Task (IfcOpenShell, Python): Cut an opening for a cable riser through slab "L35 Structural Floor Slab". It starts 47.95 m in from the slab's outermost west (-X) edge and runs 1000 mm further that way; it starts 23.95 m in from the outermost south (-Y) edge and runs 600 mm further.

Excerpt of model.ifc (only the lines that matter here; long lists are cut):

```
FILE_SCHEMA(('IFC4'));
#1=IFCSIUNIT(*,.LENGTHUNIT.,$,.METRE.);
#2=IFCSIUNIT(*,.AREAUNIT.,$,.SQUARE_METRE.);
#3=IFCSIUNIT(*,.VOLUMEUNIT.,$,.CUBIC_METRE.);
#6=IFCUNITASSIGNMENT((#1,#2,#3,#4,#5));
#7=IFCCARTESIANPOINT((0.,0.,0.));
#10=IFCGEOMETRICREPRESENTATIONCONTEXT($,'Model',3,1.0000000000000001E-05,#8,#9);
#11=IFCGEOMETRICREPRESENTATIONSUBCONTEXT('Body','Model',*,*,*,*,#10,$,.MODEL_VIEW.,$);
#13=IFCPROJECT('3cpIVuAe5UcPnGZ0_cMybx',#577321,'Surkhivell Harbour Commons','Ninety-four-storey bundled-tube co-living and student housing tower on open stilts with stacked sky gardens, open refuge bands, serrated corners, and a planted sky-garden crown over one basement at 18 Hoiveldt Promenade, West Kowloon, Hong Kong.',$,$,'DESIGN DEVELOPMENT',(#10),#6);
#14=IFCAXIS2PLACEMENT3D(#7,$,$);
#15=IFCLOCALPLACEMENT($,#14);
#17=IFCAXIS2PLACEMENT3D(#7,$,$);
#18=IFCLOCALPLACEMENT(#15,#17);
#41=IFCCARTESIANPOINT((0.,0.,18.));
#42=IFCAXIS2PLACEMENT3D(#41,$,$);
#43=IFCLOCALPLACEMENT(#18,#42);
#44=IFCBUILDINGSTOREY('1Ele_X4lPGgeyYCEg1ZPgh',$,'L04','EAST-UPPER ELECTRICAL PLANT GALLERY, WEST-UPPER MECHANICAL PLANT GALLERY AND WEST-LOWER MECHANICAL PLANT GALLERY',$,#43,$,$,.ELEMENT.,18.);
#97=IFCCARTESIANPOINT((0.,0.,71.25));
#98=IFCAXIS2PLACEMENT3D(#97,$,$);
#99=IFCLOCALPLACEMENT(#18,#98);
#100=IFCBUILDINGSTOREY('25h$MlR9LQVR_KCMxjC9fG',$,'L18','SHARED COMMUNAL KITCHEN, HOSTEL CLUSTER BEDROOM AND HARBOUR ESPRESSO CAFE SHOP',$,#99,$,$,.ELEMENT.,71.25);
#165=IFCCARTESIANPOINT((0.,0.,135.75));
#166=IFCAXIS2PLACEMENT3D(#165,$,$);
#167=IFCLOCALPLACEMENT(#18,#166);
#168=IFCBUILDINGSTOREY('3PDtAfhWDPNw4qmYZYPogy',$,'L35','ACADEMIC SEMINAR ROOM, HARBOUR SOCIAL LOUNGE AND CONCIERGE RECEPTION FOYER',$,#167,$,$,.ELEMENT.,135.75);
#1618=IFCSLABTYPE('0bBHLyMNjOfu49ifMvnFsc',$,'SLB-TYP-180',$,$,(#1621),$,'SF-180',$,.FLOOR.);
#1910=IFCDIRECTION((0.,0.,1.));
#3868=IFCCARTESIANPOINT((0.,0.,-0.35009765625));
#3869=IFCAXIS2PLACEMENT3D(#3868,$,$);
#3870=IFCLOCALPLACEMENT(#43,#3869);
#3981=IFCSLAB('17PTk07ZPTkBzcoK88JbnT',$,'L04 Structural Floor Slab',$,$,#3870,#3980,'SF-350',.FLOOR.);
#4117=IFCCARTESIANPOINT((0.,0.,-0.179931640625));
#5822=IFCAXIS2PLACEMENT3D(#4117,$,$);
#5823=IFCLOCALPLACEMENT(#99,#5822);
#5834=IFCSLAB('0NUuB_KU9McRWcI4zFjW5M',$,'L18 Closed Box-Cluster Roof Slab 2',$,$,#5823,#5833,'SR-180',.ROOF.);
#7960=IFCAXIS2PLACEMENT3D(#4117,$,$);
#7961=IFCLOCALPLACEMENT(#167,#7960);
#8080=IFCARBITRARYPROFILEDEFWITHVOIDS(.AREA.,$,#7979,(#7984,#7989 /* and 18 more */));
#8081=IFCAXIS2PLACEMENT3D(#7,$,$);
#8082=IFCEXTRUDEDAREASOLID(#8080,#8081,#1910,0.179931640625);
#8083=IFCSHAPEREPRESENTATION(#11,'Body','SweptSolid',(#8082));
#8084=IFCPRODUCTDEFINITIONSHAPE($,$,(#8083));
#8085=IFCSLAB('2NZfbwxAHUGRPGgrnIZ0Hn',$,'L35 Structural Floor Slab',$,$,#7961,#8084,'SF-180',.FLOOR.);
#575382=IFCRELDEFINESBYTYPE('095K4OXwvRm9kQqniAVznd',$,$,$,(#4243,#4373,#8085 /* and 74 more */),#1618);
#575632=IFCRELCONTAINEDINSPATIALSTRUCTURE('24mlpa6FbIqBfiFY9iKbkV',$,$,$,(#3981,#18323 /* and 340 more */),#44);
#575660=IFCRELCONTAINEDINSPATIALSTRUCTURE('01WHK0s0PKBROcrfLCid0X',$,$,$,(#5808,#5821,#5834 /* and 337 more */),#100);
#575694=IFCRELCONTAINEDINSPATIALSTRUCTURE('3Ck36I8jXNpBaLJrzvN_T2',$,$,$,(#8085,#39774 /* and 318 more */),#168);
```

```python
import numpy as np
import ifcopenshell
import ifcopenshell.api.feature
import ifcopenshell.api.geometry
import ifcopenshell.api.root
import ifcopenshell.geom
import ifcopenshell.util.placement
import ifcopenshell.util.representation
import ifcopenshell.util.shape
import ifcopenshell.util.unit

model = ifcopenshell.open("model.ifc")
unit_scale = ifcopenshell.util.unit.calculate_unit_scale(model)
settings = ifcopenshell.geom.settings()


def volume(element):
    """Net volume in cubic metres, openings subtracted."""
    shape = ifcopenshell.geom.create_shape(settings, element)
    return ifcopenshell.util.shape.get_volume(shape.geometry)


slab = model.by_id(8085)
before = volume(slab)

# Extent in the slab's own axes, in metres. The edges named are its -X and -Y sides.
slab_shape = ifcopenshell.geom.create_shape(settings, slab)
vertices = ifcopenshell.util.shape.get_vertices(slab_shape.geometry)
x_min, y_min, bottom = vertices.min(axis=0)
top = vertices[:, 2].max()

opening = ifcopenshell.api.root.create_entity(model, ifc_class="IfcOpeningElement", name="Cable riser opening", predefined_type="OPENING")
context = ifcopenshell.util.representation.get_context(model, "Model", "Body", "MODEL_VIEW")
width, depth = 1, 0.6
outline = [(0.0, 0.0), (width, 0.0), (width, depth), (0.0, depth), (0.0, 0.0)]
# Overshoot both faces by 50 mm so the cut is clean.
shape = ifcopenshell.api.geometry.add_slab_representation(
    model, context=context, depth=top - bottom + 0.1, polyline=outline
)
ifcopenshell.api.geometry.assign_representation(model, product=opening, representation=shape)

matrix = ifcopenshell.util.placement.get_local_placement(slab.ObjectPlacement)
matrix[:, 3] = matrix @ np.append(np.array([x_min + 47.95, y_min + 23.95, bottom - 0.05]) / unit_scale, 1.0)
ifcopenshell.api.geometry.edit_object_placement(model, product=opening, matrix=matrix, is_si=False)
ifcopenshell.api.feature.add_feature(model, feature=opening, element=slab)

after = volume(slab)

print(f"slab volume {before:.3f} -> {after:.3f} m3")

model.write("model_v2.ifc")
```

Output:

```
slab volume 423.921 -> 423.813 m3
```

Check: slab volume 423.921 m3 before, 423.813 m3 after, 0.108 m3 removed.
